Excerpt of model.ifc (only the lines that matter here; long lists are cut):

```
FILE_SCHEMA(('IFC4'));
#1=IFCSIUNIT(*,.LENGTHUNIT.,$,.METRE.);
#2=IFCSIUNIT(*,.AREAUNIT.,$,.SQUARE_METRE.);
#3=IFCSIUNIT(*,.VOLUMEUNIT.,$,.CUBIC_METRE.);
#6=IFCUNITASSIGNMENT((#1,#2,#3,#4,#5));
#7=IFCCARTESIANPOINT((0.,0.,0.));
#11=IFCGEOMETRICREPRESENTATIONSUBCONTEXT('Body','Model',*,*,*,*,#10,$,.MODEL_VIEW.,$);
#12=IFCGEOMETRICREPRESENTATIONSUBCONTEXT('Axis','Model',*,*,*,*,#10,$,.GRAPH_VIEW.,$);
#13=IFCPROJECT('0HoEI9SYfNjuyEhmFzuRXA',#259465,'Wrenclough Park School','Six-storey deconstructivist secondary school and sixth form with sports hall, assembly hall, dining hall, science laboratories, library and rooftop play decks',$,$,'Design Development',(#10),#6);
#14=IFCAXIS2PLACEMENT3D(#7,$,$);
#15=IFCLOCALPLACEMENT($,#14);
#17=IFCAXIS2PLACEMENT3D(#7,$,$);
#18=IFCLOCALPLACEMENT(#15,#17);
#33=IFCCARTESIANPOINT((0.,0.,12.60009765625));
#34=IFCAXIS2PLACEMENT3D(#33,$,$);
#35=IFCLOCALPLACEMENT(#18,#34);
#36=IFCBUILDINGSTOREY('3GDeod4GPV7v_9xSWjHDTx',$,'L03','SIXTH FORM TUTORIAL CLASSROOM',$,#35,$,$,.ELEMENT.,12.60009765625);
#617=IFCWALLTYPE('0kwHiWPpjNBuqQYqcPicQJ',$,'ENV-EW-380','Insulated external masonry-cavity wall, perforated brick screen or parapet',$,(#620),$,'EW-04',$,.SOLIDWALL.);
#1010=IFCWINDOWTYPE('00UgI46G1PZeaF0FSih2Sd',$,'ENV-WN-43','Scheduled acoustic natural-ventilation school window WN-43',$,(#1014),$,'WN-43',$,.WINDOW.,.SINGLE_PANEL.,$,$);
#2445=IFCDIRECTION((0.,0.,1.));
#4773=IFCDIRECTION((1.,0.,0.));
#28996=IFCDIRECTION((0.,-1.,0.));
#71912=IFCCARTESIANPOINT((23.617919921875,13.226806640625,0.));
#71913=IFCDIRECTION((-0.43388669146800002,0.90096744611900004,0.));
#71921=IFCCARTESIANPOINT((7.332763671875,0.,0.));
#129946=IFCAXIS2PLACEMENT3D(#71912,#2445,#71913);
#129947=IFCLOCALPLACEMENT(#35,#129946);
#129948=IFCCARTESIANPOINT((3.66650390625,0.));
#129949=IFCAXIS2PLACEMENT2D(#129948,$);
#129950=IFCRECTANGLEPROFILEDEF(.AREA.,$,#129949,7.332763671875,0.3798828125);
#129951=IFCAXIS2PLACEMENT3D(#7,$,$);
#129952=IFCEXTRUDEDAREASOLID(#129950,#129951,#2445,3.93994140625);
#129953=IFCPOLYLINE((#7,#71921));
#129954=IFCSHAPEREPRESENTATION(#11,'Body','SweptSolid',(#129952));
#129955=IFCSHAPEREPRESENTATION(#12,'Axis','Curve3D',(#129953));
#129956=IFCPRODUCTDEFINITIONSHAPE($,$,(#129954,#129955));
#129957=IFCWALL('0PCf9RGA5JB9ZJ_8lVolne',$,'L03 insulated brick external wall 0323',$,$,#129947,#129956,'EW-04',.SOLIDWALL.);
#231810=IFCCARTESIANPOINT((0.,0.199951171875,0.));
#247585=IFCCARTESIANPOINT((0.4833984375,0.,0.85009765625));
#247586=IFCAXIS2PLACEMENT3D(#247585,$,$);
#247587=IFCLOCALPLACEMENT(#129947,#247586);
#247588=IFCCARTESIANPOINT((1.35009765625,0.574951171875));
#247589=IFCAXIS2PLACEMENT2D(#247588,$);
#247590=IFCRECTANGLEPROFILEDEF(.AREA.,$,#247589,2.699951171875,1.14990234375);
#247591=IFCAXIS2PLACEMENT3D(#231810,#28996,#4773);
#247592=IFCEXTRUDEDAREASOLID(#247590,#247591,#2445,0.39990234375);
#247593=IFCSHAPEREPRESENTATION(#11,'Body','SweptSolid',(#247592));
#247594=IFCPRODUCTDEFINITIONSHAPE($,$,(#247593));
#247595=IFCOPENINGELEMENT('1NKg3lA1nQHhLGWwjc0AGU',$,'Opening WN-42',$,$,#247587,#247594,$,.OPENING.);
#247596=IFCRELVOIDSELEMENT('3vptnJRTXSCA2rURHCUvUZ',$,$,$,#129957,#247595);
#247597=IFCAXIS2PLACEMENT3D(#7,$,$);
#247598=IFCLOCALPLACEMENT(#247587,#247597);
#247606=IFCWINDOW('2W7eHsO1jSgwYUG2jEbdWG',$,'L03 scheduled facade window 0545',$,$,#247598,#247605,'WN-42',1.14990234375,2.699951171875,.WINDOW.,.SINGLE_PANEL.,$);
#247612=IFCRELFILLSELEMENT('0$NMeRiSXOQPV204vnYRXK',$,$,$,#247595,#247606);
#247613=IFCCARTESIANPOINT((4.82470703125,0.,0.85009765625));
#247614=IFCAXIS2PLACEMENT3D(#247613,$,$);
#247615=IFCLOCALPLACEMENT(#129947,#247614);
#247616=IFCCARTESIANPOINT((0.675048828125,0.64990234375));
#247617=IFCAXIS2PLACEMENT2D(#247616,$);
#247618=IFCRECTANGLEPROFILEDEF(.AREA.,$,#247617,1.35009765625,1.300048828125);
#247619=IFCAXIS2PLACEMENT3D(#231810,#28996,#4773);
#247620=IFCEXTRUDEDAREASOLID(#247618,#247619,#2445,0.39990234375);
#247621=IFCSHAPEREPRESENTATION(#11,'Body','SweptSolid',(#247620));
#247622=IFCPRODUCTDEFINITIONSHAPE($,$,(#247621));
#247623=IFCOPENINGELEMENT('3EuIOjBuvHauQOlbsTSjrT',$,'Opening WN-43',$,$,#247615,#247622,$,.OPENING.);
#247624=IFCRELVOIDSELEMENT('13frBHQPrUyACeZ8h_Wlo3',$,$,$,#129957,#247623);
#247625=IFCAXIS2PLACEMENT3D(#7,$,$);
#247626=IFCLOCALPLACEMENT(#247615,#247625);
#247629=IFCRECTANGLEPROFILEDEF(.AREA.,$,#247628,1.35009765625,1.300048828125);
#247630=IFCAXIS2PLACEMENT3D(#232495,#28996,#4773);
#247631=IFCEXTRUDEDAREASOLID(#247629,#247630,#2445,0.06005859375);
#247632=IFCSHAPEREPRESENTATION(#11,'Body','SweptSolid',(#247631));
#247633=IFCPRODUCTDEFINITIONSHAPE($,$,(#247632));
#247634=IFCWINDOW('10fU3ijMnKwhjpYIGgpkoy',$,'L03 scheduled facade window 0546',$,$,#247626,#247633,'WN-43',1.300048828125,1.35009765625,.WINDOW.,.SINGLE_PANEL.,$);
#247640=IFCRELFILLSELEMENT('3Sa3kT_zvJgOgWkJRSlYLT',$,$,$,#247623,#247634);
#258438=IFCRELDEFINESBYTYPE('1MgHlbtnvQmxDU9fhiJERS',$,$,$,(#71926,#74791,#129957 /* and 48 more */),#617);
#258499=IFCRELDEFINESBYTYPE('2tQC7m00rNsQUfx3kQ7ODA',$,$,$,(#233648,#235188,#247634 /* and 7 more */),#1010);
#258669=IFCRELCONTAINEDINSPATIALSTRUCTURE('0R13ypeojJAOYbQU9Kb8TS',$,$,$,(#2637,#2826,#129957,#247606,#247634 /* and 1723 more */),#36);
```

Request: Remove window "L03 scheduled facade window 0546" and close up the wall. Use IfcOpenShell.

```python
import ifcopenshell
import ifcopenshell.api.feature
import ifcopenshell.api.root
import ifcopenshell.geom
import ifcopenshell.util.shape

model = ifcopenshell.open("model.ifc")
settings = ifcopenshell.geom.settings()


def volume(element):
    """Net volume in cubic metres, openings subtracted."""
    shape = ifcopenshell.geom.create_shape(settings, element)
    return ifcopenshell.util.shape.get_volume(shape.geometry)


window = model.by_guid("10fU3ijMnKwhjpYIGgpkoy")
opening = window.FillsVoids[0].RelatingOpeningElement
wall = opening.VoidsElements[0].RelatingBuildingElement
before = volume(wall)

ifcopenshell.api.root.remove_product(model, product=window)
ifcopenshell.api.feature.remove_feature(model, feature=opening)

after = volume(wall)

print(f"wall volume {before:.3f} -> {after:.3f} m3")

model.write("model-out.ifc")
```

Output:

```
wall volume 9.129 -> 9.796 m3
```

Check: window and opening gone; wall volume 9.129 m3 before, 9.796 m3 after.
